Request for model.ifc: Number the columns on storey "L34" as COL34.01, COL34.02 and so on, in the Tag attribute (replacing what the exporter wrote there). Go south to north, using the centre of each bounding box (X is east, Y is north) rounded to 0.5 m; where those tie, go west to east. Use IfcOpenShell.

First a look at what the model holds.

```python
import ifcopenshell
import ifcopenshell.util.element
import ifcopenshell.util.placement

model = ifcopenshell.open("model.ifc")
print(model.schema)
storey = next(s for s in model.by_type("IfcBuildingStorey") if s.Name == "L34")
columns = [e for e in ifcopenshell.util.element.get_decomposition(storey) if e.is_a("IfcColumn")]
for e in sorted(columns, key=lambda e: e.id()):
    origin = ifcopenshell.util.placement.get_local_placement(e.ObjectPlacement)[:3, 3]
    print(e.id(), e.Tag, e.Name, origin.round(2) + 0.0, sep=" | ")
```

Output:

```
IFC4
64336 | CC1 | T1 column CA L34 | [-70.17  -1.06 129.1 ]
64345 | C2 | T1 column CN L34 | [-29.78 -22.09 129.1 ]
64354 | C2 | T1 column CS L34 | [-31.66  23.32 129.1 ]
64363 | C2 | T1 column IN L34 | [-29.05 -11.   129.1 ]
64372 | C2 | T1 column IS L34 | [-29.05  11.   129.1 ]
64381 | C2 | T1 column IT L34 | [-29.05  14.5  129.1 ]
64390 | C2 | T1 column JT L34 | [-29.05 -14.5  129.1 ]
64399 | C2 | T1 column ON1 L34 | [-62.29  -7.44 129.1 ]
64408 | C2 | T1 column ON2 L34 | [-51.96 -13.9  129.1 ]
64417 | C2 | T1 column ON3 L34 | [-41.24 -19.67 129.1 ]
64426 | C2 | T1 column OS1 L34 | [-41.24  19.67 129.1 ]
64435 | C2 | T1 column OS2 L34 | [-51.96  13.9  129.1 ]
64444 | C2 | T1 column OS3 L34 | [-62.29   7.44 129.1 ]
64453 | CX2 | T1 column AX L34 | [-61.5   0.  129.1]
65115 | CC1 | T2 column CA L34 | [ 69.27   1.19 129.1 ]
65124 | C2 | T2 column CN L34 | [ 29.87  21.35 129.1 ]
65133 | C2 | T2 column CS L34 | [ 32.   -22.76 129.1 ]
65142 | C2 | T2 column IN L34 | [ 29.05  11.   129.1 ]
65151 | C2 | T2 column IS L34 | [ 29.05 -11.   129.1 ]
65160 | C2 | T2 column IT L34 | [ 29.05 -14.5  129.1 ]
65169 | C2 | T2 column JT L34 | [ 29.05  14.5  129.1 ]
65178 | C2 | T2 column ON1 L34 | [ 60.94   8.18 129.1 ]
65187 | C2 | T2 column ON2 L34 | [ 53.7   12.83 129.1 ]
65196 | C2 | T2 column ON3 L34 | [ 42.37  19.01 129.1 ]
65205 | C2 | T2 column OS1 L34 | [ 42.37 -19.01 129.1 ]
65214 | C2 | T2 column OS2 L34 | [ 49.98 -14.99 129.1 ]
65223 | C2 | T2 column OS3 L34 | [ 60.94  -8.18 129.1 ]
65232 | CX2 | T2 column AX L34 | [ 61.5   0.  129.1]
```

```python
import ifcopenshell
import ifcopenshell.geom
import ifcopenshell.util.element
import ifcopenshell.util.shape

model = ifcopenshell.open("model.ifc")
settings = ifcopenshell.geom.settings()
settings.set("use-world-coords", True)


def centre(element):
    shape = ifcopenshell.geom.create_shape(settings, element)
    return ifcopenshell.util.shape.get_bbox_centroid(shape.geometry)


storey = next(s for s in model.by_type("IfcBuildingStorey") if s.Name == "L34")
columns = [e for e in ifcopenshell.util.element.get_decomposition(storey) if e.is_a("IfcColumn")]

# Insertion points can sit at a corner or the storey origin, so sort by the geometry (in metres).
centres = {e: centre(e) for e in columns}
columns.sort(key=lambda e: (round(centres[e][1] / 0.5), centres[e][0]))

for i, e in enumerate(columns, start=1):
    number = f"COL34.{i:02d}"
    e.Tag = number
    print(e.id(), number)

model.write("model_v2.ifc")
```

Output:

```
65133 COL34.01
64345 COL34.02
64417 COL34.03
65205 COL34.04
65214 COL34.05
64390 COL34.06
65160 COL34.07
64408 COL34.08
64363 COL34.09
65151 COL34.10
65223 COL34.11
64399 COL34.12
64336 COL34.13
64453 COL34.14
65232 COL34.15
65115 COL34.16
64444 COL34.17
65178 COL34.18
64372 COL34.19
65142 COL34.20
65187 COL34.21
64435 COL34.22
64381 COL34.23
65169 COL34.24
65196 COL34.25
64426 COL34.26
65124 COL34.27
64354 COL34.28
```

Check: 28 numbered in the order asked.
